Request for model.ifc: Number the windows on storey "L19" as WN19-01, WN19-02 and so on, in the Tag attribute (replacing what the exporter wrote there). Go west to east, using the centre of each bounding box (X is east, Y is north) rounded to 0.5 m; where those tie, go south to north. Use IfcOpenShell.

First a look at what the model holds.

```python
import ifcopenshell
import ifcopenshell.util.element
import ifcopenshell.util.placement

model = ifcopenshell.open("model.ifc")
print(model.schema)
storey = next(s for s in model.by_type("IfcBuildingStorey") if s.Name == "L19")
windows = [e for e in ifcopenshell.util.element.get_decomposition(storey) if e.is_a("IfcWindow")]
for e in sorted(windows, key=lambda e: e.id()):
    origin = ifcopenshell.util.placement.get_local_placement(e.ObjectPlacement)[:3, 3]
    print(e.id(), e.Tag, e.Name, origin.round(2) + 0.0, sep=" | ")
```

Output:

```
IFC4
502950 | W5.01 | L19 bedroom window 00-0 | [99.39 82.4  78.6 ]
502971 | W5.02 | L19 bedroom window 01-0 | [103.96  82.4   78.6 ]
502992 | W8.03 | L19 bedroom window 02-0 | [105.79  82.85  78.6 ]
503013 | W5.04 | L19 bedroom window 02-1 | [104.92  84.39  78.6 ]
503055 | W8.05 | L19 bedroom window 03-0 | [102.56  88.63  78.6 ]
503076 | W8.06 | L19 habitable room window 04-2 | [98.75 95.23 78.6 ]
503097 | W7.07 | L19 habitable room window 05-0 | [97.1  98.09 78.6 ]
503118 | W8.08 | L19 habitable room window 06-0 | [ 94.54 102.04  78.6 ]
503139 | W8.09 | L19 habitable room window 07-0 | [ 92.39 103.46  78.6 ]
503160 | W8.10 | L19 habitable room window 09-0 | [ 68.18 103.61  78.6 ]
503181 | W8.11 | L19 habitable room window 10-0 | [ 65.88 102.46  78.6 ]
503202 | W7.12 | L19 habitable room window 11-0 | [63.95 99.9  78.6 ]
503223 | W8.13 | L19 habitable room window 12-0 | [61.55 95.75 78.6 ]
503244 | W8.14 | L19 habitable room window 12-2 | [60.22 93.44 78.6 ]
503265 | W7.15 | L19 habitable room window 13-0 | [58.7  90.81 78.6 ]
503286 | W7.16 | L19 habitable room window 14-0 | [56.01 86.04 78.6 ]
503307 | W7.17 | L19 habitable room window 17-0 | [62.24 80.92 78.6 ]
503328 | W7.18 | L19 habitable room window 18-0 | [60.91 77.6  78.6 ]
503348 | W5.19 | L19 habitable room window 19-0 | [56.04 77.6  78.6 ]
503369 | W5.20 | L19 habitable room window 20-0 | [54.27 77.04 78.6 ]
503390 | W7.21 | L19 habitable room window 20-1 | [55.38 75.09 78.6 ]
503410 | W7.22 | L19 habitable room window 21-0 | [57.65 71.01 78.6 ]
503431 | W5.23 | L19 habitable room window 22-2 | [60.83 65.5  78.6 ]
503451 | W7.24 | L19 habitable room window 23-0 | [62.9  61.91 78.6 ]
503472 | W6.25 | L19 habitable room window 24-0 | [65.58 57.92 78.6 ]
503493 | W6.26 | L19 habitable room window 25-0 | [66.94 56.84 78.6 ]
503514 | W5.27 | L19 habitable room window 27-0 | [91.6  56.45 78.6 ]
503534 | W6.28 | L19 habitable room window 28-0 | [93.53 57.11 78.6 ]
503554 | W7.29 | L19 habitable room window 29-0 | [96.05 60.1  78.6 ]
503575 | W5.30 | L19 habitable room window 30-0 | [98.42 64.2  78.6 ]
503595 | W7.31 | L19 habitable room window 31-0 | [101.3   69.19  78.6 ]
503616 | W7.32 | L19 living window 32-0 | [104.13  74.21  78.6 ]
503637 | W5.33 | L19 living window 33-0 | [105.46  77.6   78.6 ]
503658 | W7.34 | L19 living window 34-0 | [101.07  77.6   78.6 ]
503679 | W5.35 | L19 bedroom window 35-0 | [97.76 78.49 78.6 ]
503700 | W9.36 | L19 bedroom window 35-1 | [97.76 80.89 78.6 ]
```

```python
import ifcopenshell
import ifcopenshell.geom
import ifcopenshell.util.element
import ifcopenshell.util.shape

model = ifcopenshell.open("model.ifc")
settings = ifcopenshell.geom.settings()
settings.set("use-world-coords", True)


def centre(element):
    shape = ifcopenshell.geom.create_shape(settings, element)
    return ifcopenshell.util.shape.get_bbox_centroid(shape.geometry)


storey = next(s for s in model.by_type("IfcBuildingStorey") if s.Name == "L19")
windows = [e for e in ifcopenshell.util.element.get_decomposition(storey) if e.is_a("IfcWindow")]

# Insertion points can sit at a corner or the storey origin, so sort by the geometry (in metres).
centres = {e: centre(e) for e in windows}
windows.sort(key=lambda e: (round(centres[e][0] / 0.5), centres[e][1]))

for i, e in enumerate(windows, start=1):
    number = f"WN19-{i:02d}"
    e.Tag = number
    print(e.id(), number)

model.write("model-out.ifc")
```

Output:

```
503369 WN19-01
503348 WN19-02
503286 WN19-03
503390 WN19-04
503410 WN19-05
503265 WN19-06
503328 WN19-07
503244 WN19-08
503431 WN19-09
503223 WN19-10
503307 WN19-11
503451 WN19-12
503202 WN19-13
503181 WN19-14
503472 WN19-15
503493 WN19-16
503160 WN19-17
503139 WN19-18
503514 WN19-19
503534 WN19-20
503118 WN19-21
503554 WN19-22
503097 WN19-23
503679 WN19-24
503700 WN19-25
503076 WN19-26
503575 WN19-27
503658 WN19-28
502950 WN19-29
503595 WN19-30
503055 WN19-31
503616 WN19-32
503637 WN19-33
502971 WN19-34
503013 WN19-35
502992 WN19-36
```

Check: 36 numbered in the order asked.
